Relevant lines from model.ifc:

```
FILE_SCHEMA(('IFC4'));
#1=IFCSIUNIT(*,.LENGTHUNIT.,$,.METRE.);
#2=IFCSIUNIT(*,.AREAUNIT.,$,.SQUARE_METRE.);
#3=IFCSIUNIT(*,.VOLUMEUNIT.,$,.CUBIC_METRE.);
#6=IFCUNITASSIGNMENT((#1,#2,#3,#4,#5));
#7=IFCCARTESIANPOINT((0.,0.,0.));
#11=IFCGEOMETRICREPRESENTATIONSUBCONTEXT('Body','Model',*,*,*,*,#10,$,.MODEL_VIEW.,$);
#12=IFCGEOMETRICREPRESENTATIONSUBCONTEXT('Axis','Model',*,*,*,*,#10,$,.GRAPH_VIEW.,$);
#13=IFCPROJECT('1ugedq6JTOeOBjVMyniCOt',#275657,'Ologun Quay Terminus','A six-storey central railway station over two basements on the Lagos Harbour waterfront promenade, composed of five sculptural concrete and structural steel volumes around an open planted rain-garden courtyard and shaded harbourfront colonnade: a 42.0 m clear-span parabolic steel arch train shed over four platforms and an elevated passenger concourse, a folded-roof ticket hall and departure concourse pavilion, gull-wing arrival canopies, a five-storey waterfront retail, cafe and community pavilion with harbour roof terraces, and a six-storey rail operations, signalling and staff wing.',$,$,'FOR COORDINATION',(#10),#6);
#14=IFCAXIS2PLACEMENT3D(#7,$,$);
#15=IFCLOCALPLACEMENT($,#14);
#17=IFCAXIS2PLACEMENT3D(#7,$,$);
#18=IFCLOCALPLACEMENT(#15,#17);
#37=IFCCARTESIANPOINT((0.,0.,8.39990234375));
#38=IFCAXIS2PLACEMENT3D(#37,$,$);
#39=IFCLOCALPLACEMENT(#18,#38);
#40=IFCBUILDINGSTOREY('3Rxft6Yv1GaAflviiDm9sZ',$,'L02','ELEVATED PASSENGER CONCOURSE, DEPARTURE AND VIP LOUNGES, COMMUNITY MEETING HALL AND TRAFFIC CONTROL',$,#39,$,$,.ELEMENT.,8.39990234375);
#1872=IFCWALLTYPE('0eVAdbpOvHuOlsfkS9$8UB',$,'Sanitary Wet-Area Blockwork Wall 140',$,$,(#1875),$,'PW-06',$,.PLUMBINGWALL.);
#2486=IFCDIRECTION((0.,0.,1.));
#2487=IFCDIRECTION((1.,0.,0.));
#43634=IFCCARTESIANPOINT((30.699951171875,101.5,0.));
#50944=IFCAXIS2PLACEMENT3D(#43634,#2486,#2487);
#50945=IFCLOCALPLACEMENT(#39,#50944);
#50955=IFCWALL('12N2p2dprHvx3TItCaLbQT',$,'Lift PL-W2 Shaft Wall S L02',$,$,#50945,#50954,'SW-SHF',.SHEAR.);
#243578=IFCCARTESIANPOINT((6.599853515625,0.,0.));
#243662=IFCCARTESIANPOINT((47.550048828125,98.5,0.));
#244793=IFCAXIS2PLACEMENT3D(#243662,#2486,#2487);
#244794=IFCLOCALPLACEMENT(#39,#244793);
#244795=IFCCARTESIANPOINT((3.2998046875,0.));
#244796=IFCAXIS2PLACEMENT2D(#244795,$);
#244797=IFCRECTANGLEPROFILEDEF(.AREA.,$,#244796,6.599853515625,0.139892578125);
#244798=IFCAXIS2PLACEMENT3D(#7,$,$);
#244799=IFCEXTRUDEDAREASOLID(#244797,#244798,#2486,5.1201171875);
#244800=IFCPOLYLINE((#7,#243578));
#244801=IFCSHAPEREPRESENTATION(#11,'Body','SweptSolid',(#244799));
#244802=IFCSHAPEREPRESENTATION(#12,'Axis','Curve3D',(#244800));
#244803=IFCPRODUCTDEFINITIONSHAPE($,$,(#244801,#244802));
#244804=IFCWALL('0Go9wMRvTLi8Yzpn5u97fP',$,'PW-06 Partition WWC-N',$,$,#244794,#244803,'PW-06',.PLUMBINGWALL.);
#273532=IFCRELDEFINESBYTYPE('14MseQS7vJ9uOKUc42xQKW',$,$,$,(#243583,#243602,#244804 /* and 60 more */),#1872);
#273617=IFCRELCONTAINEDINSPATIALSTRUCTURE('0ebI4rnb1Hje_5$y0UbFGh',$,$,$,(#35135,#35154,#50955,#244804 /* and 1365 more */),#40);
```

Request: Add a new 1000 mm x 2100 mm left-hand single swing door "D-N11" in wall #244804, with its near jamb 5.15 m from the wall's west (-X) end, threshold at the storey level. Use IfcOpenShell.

```python
import numpy as np
import ifcopenshell
import ifcopenshell.api.feature
import ifcopenshell.api.geometry
import ifcopenshell.api.root
import ifcopenshell.api.spatial
import ifcopenshell.geom
import ifcopenshell.util.element
import ifcopenshell.util.placement
import ifcopenshell.util.representation
import ifcopenshell.util.shape
import ifcopenshell.util.unit

model = ifcopenshell.open("model.ifc")
unit_scale = ifcopenshell.util.unit.calculate_unit_scale(model)
settings = ifcopenshell.geom.settings()


def volume(element):
    """Net volume in cubic metres, openings subtracted."""
    shape = ifcopenshell.geom.create_shape(settings, element)
    return ifcopenshell.util.shape.get_volume(shape.geometry)


wall = model.by_guid("0Go9wMRvTLi8Yzpn5u97fP")
storey = ifcopenshell.util.element.get_container(wall, ifc_class="IfcBuildingStorey")
context = ifcopenshell.util.representation.get_context(model, "Model", "Body", "MODEL_VIEW")
before = volume(wall)

width, height, from_end, sill = 1, 2.1, 5.15, 0.0  # metres

# The wall runs along its own X axis, and the end named is its -X end.
wall_shape = ifcopenshell.geom.create_shape(settings, wall)
x, y, z = ifcopenshell.util.shape.get_vertices(wall_shape.geometry).T
start = x.min() + from_end
face, thickness = float(y.min()), float(y.max() - y.min())
wall_matrix = ifcopenshell.util.placement.get_local_placement(wall.ObjectPlacement)
level = ifcopenshell.util.placement.get_local_placement(storey.ObjectPlacement)[2, 3]


def in_wall(x, y):
    """Placement at x, y metres in the wall's axes, at sill height."""
    matrix = wall_matrix.copy()
    matrix[:, 3] = wall_matrix @ np.array([x / unit_scale, y / unit_scale, 0.0, 1.0])
    matrix[2, 3] = level + sill / unit_scale
    return matrix


# Opening: a box that overshoots both wall faces by 50 mm.
opening = ifcopenshell.api.root.create_entity(model, ifc_class="IfcOpeningElement", predefined_type="OPENING")
box = ifcopenshell.api.geometry.add_wall_representation(
    model, context=context, length=width, height=height, thickness=thickness + 0.1
)
ifcopenshell.api.geometry.assign_representation(model, product=opening, representation=box)
ifcopenshell.api.geometry.edit_object_placement(model, product=opening, matrix=in_wall(start, face - 0.05), is_si=False)
ifcopenshell.api.feature.add_feature(model, feature=opening, element=wall)

door = ifcopenshell.api.root.create_entity(model, ifc_class="IfcDoor", name="D-N11", predefined_type="DOOR")
door.OverallWidth, door.OverallHeight = width / unit_scale, height / unit_scale
door.OperationType = "SINGLE_SWING_LEFT"
body = ifcopenshell.api.geometry.add_door_representation(
    model,
    context=context,
    overall_width=door.OverallWidth,
    overall_height=door.OverallHeight,
    operation_type="SINGLE_SWING_LEFT",
    lining_properties={"LiningDepth": thickness / unit_scale, "ThresholdDepth": thickness / unit_scale},
)
ifcopenshell.api.geometry.assign_representation(model, product=door, representation=body)
ifcopenshell.api.spatial.assign_container(model, products=[door], relating_structure=storey)
ifcopenshell.api.feature.add_filling(model, opening=opening, element=door)

# The lining spans the wall, so the door starts at the wall face.
ifcopenshell.api.geometry.edit_object_placement(model, product=door, matrix=in_wall(start, face), is_si=False)

after = volume(wall)

print(f"wall volume {before:.3f} -> {after:.3f} m3")

model.write("model_v2.ifc")
```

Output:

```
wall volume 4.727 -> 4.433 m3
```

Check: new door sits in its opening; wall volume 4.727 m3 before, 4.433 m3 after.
